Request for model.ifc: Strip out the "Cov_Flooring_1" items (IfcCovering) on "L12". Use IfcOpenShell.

First a look at what the model holds.

```python
import ifcopenshell
import ifcopenshell.util.element

model = ifcopenshell.open("model.ifc")
print(model.schema)
storey = next(s for s in model.by_type("IfcBuildingStorey") if s.Name == "L12")
coverings = [e for e in ifcopenshell.util.element.get_decomposition(storey) if e.is_a("IfcCovering")]
seen = {}
for e in coverings:
    element_type = ifcopenshell.util.element.get_type(e)
    name = element_type.Name if element_type not in (None, e) else None
    seen[name] = seen.get(name, 0) + 1
for name, count in sorted(seen.items(), key=str):
    print(count, "x", name)
```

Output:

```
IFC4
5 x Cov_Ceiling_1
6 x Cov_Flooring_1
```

```python
import ifcopenshell
import ifcopenshell.api.root
import ifcopenshell.util.element

model = ifcopenshell.open("model.ifc")

storey = next(s for s in model.by_type("IfcBuildingStorey") if s.Name == "L12")
coverings = [e for e in ifcopenshell.util.element.get_decomposition(storey) if e.is_a("IfcCovering")]
targets = [e for e in coverings if (t := ifcopenshell.util.element.get_type(e)) not in (None, e) and t.Name == "Cov_Flooring_1"]

for e in targets:
    ifcopenshell.api.root.remove_product(model, product=e)
print(len(targets), "removed")

model.write("model_edited.ifc")
```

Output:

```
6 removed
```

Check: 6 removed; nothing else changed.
